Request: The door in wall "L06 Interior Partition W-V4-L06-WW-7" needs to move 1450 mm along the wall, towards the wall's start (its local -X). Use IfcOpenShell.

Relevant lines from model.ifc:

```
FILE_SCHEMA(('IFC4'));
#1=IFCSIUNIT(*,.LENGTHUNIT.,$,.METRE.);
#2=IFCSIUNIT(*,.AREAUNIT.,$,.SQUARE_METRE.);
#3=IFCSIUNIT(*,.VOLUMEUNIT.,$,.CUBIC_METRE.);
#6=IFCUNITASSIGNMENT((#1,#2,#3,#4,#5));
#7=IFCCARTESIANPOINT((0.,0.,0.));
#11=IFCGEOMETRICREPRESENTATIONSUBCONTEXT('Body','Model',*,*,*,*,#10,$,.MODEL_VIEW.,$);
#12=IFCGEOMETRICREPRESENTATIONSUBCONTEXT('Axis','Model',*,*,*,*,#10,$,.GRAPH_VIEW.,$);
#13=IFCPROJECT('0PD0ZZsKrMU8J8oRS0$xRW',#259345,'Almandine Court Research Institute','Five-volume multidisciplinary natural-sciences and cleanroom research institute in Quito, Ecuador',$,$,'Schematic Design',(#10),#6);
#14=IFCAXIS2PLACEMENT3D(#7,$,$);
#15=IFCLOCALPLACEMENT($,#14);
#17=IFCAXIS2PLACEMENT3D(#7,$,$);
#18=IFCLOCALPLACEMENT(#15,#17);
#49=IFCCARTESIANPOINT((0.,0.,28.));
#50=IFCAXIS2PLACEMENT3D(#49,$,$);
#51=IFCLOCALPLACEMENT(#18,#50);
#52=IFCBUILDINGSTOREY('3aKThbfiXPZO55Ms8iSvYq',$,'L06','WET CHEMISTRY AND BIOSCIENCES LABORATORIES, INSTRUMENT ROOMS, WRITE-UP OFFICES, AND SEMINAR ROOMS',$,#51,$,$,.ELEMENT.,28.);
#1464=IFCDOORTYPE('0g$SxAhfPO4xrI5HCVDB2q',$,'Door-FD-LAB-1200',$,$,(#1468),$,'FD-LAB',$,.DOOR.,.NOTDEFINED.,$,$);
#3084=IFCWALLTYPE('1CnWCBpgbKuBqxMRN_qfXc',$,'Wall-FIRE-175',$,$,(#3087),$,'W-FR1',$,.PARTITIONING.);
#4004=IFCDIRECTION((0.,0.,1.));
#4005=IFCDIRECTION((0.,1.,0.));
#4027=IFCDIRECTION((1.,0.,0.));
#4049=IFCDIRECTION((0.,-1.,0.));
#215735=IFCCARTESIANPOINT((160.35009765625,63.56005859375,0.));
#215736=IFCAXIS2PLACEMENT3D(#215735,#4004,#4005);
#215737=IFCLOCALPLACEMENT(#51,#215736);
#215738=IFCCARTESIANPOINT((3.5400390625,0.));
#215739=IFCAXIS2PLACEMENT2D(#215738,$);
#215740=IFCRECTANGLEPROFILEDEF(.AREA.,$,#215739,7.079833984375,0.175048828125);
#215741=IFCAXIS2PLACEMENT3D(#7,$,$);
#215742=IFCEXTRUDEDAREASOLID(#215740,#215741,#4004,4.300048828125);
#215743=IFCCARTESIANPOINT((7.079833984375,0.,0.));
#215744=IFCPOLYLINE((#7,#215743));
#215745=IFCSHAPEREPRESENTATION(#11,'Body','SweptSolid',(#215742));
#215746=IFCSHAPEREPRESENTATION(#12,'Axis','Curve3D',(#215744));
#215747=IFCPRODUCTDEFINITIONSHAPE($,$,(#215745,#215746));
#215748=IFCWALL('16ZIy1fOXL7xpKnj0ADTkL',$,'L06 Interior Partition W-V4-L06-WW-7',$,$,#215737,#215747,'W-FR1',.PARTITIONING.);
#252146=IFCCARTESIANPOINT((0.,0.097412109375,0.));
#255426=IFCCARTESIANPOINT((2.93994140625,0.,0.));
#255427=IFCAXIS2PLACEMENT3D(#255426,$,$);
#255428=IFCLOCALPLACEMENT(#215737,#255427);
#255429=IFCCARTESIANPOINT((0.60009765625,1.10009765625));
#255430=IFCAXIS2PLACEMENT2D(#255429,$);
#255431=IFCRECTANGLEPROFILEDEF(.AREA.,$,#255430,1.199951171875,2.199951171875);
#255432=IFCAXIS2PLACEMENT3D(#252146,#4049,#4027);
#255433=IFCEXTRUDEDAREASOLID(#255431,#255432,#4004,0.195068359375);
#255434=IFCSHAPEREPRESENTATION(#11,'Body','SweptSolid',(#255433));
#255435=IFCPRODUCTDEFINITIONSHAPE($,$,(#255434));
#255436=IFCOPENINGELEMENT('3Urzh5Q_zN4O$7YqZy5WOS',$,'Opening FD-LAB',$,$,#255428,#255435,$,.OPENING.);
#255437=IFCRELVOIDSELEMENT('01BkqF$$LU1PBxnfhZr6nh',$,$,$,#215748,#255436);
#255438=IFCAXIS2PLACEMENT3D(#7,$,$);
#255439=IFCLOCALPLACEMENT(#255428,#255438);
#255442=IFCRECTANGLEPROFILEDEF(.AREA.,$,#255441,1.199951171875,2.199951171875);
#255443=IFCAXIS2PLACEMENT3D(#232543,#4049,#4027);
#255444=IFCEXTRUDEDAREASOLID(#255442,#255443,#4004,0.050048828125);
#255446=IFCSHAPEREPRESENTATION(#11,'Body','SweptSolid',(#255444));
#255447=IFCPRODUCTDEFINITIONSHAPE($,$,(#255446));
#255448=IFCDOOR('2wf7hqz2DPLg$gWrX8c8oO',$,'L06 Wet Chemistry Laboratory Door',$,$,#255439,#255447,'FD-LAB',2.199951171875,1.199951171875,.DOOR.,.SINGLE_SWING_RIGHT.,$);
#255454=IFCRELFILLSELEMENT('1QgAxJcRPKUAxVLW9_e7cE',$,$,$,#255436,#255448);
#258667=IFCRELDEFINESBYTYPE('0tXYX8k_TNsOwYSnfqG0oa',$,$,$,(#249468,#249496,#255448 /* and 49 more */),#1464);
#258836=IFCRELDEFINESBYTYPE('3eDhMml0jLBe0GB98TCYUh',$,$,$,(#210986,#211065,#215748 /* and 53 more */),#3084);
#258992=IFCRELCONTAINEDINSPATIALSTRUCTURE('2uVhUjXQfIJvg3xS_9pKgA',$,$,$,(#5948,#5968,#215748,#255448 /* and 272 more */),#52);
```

```python
import ifcopenshell
import ifcopenshell.api.geometry
import ifcopenshell.util.placement

model = ifcopenshell.open("model.ifc")

door = model.by_id(255448)
opening = door.FillsVoids[0].RelatingOpeningElement
wall = opening.VoidsElements[0].RelatingBuildingElement

wall_matrix = ifcopenshell.util.placement.get_local_placement(wall.ObjectPlacement)
shift = wall_matrix[:3, 0] * -1.45
before = ifcopenshell.util.placement.get_local_placement(door.ObjectPlacement)[:3, 3].copy()

# The door is placed relative to its opening, so it follows when the opening moves.
matrix = ifcopenshell.util.placement.get_local_placement(opening.ObjectPlacement)
matrix[:3, 3] += shift
ifcopenshell.api.geometry.edit_object_placement(
    model, product=opening, matrix=matrix, is_si=False, should_transform_children=True
)

after = ifcopenshell.util.placement.get_local_placement(door.ObjectPlacement)[:3, 3]
print("door moved by", (after - before).round(3) + 0.0)

model.write("model_rev.ifc")
```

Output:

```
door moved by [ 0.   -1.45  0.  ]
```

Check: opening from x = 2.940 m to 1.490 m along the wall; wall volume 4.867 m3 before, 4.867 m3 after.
